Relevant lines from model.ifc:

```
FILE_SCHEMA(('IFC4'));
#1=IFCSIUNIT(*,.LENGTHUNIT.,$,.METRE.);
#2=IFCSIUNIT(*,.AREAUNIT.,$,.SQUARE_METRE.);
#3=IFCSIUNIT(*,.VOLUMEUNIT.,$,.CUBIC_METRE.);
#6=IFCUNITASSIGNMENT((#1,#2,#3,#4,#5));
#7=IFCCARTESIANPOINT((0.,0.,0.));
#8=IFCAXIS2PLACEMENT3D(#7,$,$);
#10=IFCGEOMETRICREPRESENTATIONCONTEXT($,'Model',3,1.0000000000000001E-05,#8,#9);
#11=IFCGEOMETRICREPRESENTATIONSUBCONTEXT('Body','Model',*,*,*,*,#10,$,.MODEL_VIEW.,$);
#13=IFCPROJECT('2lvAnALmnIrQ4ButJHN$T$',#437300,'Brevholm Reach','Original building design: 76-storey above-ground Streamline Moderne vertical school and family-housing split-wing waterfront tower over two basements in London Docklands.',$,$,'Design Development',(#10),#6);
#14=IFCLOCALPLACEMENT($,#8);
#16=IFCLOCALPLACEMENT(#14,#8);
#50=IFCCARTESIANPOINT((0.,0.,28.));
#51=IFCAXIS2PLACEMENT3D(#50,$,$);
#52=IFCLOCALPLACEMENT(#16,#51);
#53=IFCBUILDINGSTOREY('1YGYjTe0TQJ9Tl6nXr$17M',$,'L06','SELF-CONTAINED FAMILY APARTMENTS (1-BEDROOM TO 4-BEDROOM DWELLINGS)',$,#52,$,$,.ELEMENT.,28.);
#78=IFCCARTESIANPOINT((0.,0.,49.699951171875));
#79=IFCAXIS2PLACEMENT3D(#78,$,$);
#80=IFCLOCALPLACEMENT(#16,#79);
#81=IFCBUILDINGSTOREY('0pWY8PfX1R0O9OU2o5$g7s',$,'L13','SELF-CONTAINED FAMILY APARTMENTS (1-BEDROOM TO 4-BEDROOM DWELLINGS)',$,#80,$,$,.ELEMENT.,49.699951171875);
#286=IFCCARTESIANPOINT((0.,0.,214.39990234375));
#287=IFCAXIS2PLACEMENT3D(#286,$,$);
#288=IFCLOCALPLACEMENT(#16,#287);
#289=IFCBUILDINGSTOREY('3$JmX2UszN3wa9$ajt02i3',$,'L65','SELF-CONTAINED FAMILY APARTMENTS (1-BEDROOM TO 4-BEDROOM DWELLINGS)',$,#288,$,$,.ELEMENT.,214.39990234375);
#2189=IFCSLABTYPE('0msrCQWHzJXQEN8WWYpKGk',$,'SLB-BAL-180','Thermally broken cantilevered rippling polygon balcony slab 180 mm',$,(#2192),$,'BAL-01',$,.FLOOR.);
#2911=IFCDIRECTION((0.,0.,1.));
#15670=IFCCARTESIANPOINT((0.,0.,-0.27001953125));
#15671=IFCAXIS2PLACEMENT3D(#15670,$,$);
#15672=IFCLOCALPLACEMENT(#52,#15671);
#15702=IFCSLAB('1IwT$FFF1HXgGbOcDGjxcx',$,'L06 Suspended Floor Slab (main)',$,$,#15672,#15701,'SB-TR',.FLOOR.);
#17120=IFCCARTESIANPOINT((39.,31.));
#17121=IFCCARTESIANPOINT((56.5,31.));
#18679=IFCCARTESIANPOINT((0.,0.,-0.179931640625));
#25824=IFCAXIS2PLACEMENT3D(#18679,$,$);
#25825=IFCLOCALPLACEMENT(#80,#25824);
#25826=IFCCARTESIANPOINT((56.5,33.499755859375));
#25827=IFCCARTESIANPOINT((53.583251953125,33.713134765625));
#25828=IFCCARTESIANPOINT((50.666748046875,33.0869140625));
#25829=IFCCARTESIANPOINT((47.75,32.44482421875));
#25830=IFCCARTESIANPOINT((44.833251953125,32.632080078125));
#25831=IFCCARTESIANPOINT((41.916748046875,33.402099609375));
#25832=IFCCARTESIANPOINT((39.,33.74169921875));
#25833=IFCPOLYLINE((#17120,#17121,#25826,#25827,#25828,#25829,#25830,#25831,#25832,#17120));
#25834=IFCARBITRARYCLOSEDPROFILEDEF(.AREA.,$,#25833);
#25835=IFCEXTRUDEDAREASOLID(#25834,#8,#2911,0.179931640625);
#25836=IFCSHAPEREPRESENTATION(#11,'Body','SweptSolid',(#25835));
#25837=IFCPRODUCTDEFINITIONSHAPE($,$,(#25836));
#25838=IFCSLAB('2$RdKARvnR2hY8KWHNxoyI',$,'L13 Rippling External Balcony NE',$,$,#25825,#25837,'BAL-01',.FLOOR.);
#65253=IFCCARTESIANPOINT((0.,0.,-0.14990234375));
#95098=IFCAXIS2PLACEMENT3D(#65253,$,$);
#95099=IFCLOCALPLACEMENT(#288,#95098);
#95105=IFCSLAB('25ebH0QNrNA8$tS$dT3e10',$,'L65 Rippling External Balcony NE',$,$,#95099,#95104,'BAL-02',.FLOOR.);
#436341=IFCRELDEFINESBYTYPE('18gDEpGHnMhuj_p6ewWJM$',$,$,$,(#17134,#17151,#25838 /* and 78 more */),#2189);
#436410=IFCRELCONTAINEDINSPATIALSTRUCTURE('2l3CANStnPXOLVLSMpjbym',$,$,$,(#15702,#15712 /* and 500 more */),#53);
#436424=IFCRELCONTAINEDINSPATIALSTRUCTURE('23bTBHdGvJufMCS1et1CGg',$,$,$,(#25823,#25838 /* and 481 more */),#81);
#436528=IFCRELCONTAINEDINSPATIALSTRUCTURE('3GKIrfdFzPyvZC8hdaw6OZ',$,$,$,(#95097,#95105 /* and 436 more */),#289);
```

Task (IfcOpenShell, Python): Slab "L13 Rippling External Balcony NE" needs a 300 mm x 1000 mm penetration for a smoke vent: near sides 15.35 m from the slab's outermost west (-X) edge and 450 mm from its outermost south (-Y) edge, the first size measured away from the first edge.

```python
import numpy as np
import ifcopenshell
import ifcopenshell.api.feature
import ifcopenshell.api.geometry
import ifcopenshell.api.root
import ifcopenshell.geom
import ifcopenshell.util.placement
import ifcopenshell.util.representation
import ifcopenshell.util.shape
import ifcopenshell.util.unit

model = ifcopenshell.open("model.ifc")
unit_scale = ifcopenshell.util.unit.calculate_unit_scale(model)
settings = ifcopenshell.geom.settings()


def volume(element):
    """Net volume in cubic metres, openings subtracted."""
    shape = ifcopenshell.geom.create_shape(settings, element)
    return ifcopenshell.util.shape.get_volume(shape.geometry)


slab = model.by_id(25838)
before = volume(slab)

# Extent in the slab's own axes, in metres. The edges named are its -X and -Y sides.
slab_shape = ifcopenshell.geom.create_shape(settings, slab)
vertices = ifcopenshell.util.shape.get_vertices(slab_shape.geometry)
x_min, y_min, bottom = vertices.min(axis=0)
top = vertices[:, 2].max()

opening = ifcopenshell.api.root.create_entity(model, ifc_class="IfcOpeningElement", name="Smoke vent opening", predefined_type="OPENING")
context = ifcopenshell.util.representation.get_context(model, "Model", "Body", "MODEL_VIEW")
width, depth = 0.3, 1
outline = [(0.0, 0.0), (width, 0.0), (width, depth), (0.0, depth), (0.0, 0.0)]
# Overshoot both faces by 50 mm so the cut is clean.
shape = ifcopenshell.api.geometry.add_slab_representation(
    model, context=context, depth=top - bottom + 0.1, polyline=outline
)
ifcopenshell.api.geometry.assign_representation(model, product=opening, representation=shape)

matrix = ifcopenshell.util.placement.get_local_placement(slab.ObjectPlacement)
matrix[:, 3] = matrix @ np.append(np.array([x_min + 15.35, y_min + 0.45, bottom - 0.05]) / unit_scale, 1.0)
ifcopenshell.api.geometry.edit_object_placement(model, product=opening, matrix=matrix, is_si=False)
ifcopenshell.api.feature.add_feature(model, feature=opening, element=slab)

after = volume(slab)

print(f"slab volume {before:.3f} -> {after:.3f} m3")

model.write("model-out.ifc")
```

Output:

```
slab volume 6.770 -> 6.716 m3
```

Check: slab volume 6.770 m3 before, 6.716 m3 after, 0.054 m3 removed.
